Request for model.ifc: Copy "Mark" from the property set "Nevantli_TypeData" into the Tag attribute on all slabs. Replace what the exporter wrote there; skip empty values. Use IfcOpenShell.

First a look at what the model holds.

```python
import ifcopenshell
import ifcopenshell.util.element

model = ifcopenshell.open("model.ifc")
print(model.schema)
slabs = model.by_type("IfcSlab")
print(len(slabs), "slabs")
for e in slabs[:8]:
    source = ifcopenshell.util.element.get_pset(e, "Nevantli_TypeData", "Mark")
    target = e.Tag
    print(e.id(), repr(source), repr(target), sep=" | ")
```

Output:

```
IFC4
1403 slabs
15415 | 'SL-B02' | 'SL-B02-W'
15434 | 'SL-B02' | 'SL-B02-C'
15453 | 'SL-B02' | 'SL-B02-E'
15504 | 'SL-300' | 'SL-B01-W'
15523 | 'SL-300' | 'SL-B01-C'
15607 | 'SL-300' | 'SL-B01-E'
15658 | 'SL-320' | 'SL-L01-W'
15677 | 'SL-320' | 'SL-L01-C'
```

```python
import ifcopenshell
import ifcopenshell.util.element

model = ifcopenshell.open("model.ifc")

count = 0
for e in model.by_type("IfcSlab"):
    value = ifcopenshell.util.element.get_pset(e, "Nevantli_TypeData", "Mark")
    current = e.Tag
    if not value or not value.strip() or current == value:
        continue
    e.Tag = value
    count += 1

print(count, "slabs updated")

model.write("model_updated.ifc")
```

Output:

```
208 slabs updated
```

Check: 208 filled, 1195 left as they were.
